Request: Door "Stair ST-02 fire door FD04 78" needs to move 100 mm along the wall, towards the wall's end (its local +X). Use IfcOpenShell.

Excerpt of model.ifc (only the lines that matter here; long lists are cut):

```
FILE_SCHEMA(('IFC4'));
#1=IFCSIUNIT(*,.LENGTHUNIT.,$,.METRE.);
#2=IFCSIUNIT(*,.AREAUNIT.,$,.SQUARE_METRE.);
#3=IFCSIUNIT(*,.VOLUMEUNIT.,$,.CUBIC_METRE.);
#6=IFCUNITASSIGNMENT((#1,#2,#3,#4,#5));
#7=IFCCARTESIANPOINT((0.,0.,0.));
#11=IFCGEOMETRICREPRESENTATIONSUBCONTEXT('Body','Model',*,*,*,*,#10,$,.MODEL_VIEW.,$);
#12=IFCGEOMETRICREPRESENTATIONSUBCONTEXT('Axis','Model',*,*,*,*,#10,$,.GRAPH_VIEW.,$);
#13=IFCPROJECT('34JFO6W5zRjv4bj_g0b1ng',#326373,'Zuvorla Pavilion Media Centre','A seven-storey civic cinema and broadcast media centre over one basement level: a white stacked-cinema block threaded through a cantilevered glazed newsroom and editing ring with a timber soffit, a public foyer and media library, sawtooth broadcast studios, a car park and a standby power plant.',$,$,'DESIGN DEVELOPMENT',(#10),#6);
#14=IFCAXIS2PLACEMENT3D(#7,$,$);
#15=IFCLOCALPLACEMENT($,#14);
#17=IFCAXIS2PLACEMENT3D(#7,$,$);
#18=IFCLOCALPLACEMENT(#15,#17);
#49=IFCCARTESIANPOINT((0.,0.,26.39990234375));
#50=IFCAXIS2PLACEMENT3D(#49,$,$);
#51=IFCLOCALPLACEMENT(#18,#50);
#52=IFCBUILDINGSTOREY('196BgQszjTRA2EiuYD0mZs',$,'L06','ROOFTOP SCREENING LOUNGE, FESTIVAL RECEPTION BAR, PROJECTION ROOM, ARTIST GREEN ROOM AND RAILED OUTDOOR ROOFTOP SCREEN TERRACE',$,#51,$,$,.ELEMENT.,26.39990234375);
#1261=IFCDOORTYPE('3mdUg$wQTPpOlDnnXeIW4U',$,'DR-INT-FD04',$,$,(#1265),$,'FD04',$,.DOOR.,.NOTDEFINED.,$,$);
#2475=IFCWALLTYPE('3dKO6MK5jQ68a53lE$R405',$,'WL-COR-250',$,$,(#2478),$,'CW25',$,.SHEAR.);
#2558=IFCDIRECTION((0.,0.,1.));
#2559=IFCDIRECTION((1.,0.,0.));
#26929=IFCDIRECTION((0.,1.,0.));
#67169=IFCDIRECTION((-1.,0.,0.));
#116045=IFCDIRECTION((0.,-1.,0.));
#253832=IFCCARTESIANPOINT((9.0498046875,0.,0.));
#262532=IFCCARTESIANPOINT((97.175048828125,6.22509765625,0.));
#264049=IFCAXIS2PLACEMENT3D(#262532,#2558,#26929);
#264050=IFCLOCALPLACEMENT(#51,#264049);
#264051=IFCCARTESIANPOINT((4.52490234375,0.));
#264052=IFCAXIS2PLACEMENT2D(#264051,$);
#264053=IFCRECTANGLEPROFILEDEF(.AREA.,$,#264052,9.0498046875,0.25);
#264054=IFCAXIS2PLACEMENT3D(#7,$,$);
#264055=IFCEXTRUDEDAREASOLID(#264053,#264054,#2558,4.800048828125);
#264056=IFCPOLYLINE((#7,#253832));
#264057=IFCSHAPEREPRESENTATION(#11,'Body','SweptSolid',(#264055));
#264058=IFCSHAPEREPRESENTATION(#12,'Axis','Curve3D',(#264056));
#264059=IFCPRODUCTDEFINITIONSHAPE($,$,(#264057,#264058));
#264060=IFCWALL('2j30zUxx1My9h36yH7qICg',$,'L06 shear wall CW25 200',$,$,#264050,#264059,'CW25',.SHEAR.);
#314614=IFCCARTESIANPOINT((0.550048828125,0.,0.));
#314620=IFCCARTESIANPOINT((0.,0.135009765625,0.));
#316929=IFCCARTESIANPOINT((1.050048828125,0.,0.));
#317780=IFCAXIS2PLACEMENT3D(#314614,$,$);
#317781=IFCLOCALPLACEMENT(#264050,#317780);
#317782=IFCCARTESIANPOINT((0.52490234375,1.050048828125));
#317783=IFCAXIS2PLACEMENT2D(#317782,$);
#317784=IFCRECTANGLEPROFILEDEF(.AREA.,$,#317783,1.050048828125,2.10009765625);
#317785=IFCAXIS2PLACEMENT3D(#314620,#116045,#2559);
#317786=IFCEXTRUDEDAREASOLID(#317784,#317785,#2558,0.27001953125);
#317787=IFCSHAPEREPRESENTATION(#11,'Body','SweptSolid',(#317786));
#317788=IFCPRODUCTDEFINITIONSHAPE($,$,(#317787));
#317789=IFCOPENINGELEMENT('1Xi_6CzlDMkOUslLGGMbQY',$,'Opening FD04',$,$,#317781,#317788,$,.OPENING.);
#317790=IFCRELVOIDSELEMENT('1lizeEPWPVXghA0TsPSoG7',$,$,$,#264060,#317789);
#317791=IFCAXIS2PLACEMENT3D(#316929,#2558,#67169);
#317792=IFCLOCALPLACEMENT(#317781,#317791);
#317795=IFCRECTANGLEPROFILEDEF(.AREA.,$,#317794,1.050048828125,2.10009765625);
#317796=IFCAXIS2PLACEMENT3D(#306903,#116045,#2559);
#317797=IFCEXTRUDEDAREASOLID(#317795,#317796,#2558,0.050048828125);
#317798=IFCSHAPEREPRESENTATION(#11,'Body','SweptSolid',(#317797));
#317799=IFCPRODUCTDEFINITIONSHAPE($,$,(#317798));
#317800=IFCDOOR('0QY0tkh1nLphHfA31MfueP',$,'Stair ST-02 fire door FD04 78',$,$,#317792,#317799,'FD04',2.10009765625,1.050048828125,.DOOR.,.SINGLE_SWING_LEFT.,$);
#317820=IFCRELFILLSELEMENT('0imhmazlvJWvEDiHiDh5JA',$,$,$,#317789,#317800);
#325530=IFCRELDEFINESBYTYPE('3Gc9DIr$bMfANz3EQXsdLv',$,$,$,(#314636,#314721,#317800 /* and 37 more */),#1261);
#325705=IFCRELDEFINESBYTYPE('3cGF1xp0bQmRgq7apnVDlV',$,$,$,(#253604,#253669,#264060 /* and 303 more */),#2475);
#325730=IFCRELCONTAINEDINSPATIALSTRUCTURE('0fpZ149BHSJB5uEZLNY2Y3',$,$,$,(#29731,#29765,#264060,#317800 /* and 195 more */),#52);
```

```python
import ifcopenshell
import ifcopenshell.api.geometry
import ifcopenshell.util.placement
import ifcopenshell.util.unit

model = ifcopenshell.open("model.ifc")
unit_scale = ifcopenshell.util.unit.calculate_unit_scale(model)

door = model.by_guid("0QY0tkh1nLphHfA31MfueP")
opening = door.FillsVoids[0].RelatingOpeningElement
wall = opening.VoidsElements[0].RelatingBuildingElement

wall_matrix = ifcopenshell.util.placement.get_local_placement(wall.ObjectPlacement)
shift = wall_matrix[:3, 0] * 0.1 / unit_scale
before = ifcopenshell.util.placement.get_local_placement(door.ObjectPlacement)[:3, 3].copy()

# The door is placed relative to its opening, so it follows when the opening moves.
matrix = ifcopenshell.util.placement.get_local_placement(opening.ObjectPlacement)
matrix[:3, 3] += shift
ifcopenshell.api.geometry.edit_object_placement(
    model, product=opening, matrix=matrix, is_si=False, should_transform_children=True
)

after = ifcopenshell.util.placement.get_local_placement(door.ObjectPlacement)[:3, 3]
print("door moved by", (after - before).round(3) + 0.0)

model.write("model_v2.ifc")
```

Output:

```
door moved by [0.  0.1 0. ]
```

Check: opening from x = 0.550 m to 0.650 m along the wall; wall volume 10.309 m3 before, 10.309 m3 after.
